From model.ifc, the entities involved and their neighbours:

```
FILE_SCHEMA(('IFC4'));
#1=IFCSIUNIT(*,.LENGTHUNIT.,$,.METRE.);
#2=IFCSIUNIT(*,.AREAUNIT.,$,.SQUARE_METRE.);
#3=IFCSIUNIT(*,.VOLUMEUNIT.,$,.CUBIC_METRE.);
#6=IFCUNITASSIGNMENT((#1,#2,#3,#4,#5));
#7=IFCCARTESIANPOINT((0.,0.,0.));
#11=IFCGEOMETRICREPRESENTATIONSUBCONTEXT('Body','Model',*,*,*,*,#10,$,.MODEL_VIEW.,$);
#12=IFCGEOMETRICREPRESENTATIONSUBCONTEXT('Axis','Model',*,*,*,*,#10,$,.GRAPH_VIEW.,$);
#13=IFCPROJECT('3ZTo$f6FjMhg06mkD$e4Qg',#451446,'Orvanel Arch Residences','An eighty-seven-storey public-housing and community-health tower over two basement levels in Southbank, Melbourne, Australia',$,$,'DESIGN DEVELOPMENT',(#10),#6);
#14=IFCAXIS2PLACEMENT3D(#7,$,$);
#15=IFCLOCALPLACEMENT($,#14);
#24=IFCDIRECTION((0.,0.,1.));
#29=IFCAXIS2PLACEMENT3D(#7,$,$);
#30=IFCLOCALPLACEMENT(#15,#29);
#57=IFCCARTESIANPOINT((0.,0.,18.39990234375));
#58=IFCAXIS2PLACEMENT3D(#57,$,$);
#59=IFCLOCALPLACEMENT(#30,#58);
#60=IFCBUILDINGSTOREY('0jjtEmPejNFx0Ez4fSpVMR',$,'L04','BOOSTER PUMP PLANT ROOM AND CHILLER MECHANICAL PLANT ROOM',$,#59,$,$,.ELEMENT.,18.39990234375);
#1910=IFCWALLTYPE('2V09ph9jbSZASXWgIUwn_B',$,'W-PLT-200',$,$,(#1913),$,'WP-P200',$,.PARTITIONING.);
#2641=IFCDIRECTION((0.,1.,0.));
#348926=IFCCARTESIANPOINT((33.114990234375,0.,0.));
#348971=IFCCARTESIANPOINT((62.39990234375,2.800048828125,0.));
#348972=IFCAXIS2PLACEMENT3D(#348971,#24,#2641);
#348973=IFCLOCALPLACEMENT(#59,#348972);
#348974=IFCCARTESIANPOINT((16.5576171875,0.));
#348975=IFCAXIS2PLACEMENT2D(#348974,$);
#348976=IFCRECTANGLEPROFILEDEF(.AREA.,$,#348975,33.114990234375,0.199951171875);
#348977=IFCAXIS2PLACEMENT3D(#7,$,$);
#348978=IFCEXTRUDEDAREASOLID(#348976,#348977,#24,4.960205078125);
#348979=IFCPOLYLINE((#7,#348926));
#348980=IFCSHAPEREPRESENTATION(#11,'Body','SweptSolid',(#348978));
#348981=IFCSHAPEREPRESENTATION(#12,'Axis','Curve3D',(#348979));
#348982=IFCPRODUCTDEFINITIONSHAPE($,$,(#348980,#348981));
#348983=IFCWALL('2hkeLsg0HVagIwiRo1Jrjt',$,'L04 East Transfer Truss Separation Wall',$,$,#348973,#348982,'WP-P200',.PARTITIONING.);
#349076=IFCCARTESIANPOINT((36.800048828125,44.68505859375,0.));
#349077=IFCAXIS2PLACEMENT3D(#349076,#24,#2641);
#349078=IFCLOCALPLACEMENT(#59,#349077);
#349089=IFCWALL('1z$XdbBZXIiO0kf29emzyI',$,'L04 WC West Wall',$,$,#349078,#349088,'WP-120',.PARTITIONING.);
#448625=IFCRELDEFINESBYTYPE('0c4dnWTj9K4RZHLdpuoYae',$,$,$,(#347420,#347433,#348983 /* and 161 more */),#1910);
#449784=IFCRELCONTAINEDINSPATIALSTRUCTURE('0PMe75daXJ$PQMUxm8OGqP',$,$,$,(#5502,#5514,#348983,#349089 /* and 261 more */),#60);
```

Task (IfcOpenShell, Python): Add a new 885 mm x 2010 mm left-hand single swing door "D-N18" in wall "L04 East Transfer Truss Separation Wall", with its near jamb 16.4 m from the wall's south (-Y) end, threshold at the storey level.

```python
import numpy as np
import ifcopenshell
import ifcopenshell.api.feature
import ifcopenshell.api.geometry
import ifcopenshell.api.root
import ifcopenshell.api.spatial
import ifcopenshell.geom
import ifcopenshell.util.element
import ifcopenshell.util.placement
import ifcopenshell.util.representation
import ifcopenshell.util.shape
import ifcopenshell.util.unit

model = ifcopenshell.open("model.ifc")
unit_scale = ifcopenshell.util.unit.calculate_unit_scale(model)
settings = ifcopenshell.geom.settings()


def volume(element):
    """Net volume in cubic metres, openings subtracted."""
    shape = ifcopenshell.geom.create_shape(settings, element)
    return ifcopenshell.util.shape.get_volume(shape.geometry)


wall = model.by_id(348983)
storey = ifcopenshell.util.element.get_container(wall, ifc_class="IfcBuildingStorey")
context = ifcopenshell.util.representation.get_context(model, "Model", "Body", "MODEL_VIEW")
before = volume(wall)

width, height, from_end, sill = 0.885, 2.01, 16.4, 0.0  # metres

# The wall runs along its own X axis, and the end named is its -X end.
wall_shape = ifcopenshell.geom.create_shape(settings, wall)
x, y, z = ifcopenshell.util.shape.get_vertices(wall_shape.geometry).T
start = x.min() + from_end
face, thickness = float(y.min()), float(y.max() - y.min())
wall_matrix = ifcopenshell.util.placement.get_local_placement(wall.ObjectPlacement)
level = ifcopenshell.util.placement.get_local_placement(storey.ObjectPlacement)[2, 3]


def in_wall(x, y):
    """Placement at x, y metres in the wall's axes, at sill height."""
    matrix = wall_matrix.copy()
    matrix[:, 3] = wall_matrix @ np.array([x / unit_scale, y / unit_scale, 0.0, 1.0])
    matrix[2, 3] = level + sill / unit_scale
    return matrix


# Opening: a box that overshoots both wall faces by 50 mm.
opening = ifcopenshell.api.root.create_entity(model, ifc_class="IfcOpeningElement", predefined_type="OPENING")
box = ifcopenshell.api.geometry.add_wall_representation(
    model, context=context, length=width, height=height, thickness=thickness + 0.1
)
ifcopenshell.api.geometry.assign_representation(model, product=opening, representation=box)
ifcopenshell.api.geometry.edit_object_placement(model, product=opening, matrix=in_wall(start, face - 0.05), is_si=False)
ifcopenshell.api.feature.add_feature(model, feature=opening, element=wall)

door = ifcopenshell.api.root.create_entity(model, ifc_class="IfcDoor", name="D-N18", predefined_type="DOOR")
door.OverallWidth, door.OverallHeight = width / unit_scale, height / unit_scale
door.OperationType = "SINGLE_SWING_LEFT"
body = ifcopenshell.api.geometry.add_door_representation(
    model,
    context=context,
    overall_width=door.OverallWidth,
    overall_height=door.OverallHeight,
    operation_type="SINGLE_SWING_LEFT",
    lining_properties={"LiningDepth": thickness / unit_scale, "ThresholdDepth": thickness / unit_scale},
)
ifcopenshell.api.geometry.assign_representation(model, product=door, representation=body)
ifcopenshell.api.spatial.assign_container(model, products=[door], relating_structure=storey)
ifcopenshell.api.feature.add_filling(model, opening=opening, element=door)

# The lining spans the wall, so the door starts at the wall face.
ifcopenshell.api.geometry.edit_object_placement(model, product=door, matrix=in_wall(start, face), is_si=False)

after = volume(wall)

print(f"wall volume {before:.3f} -> {after:.3f} m3")

model.write("model_updated.ifc")
```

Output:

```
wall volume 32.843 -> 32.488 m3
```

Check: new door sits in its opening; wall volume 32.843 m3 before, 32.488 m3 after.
